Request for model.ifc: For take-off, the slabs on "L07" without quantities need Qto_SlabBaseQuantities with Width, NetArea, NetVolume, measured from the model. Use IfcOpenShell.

First a look at what the model holds.

```python
import ifcopenshell
import ifcopenshell.util.element
import ifcopenshell.util.unit

model = ifcopenshell.open("model.ifc")
print(model.schema)
for unit_type in ("LENGTHUNIT", "AREAUNIT", "VOLUMEUNIT"):
    print(unit_type, ifcopenshell.util.unit.calculate_unit_scale(model, unit_type))
storey = next(s for s in model.by_type("IfcBuildingStorey") if s.Name == "L07")
slabs = [e for e in ifcopenshell.util.element.get_decomposition(storey) if e.is_a("IfcSlab")]
for e in sorted(slabs, key=lambda e: e.id()):
    print(e.id(), e.is_a(), e.Name, list(ifcopenshell.util.element.get_psets(e, qtos_only=True)), sep=" | ")
```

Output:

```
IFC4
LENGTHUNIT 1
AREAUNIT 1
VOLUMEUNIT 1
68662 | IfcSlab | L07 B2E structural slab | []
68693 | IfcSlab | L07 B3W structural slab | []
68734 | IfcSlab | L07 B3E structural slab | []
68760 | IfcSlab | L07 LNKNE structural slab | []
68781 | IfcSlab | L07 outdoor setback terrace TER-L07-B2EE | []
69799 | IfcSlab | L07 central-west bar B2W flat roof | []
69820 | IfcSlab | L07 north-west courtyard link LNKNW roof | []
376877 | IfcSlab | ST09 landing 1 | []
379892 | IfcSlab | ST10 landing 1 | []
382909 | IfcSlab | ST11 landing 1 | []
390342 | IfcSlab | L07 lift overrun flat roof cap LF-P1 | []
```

```python
import ifcopenshell
import ifcopenshell.api.pset
import ifcopenshell.geom
import ifcopenshell.util.element
import ifcopenshell.util.shape
import ifcopenshell.util.unit

model = ifcopenshell.open("model.ifc")
unit_scale = ifcopenshell.util.unit.calculate_unit_scale(model)
area_scale = ifcopenshell.util.unit.calculate_unit_scale(model, "AREAUNIT")
volume_scale = ifcopenshell.util.unit.calculate_unit_scale(model, "VOLUMEUNIT")
settings = ifcopenshell.geom.settings()

storey = next(s for s in model.by_type("IfcBuildingStorey") if s.Name == "L07")
slabs = [e for e in ifcopenshell.util.element.get_decomposition(storey) if e.is_a("IfcSlab")]

for e in sorted(slabs, key=lambda e: e.id()):
    if ifcopenshell.util.element.get_psets(e, qtos_only=True, should_inherit=False):
        continue
    # Geometry comes back in metres, in the element's own axes.
    shape = ifcopenshell.geom.create_shape(settings, e)
    values = {
        "Width": ifcopenshell.util.shape.get_z(shape.geometry) / unit_scale,
        "NetArea": ifcopenshell.util.shape.get_footprint_area(shape.geometry) / area_scale,
        "NetVolume": ifcopenshell.util.shape.get_volume(shape.geometry) / volume_scale,
    }
    qto = ifcopenshell.api.pset.add_qto(model, product=e, name="Qto_SlabBaseQuantities")
    ifcopenshell.api.pset.edit_qto(model, qto=qto, properties=values)
    print(e.id(), {k: round(v, 3) for k, v in values.items()})

model.write("model_rev.ifc")
```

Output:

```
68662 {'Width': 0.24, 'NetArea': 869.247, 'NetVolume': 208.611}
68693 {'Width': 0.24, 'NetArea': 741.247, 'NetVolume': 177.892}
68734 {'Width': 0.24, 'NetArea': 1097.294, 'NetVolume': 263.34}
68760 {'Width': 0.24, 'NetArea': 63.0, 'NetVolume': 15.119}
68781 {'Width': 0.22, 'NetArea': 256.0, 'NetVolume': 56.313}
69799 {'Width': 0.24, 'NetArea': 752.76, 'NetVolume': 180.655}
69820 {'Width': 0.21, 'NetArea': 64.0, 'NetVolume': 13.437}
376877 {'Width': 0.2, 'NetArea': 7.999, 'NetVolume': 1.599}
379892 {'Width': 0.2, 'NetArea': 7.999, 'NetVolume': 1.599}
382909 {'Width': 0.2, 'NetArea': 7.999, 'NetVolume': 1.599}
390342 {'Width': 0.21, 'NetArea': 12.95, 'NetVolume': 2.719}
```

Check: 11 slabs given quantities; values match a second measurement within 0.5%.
